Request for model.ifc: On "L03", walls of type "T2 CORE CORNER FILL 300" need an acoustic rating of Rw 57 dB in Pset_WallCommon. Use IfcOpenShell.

First a look at what the model holds.

```python
import ifcopenshell
import ifcopenshell.util.element

model = ifcopenshell.open("model.ifc")
print(model.schema)
storey = next(s for s in model.by_type("IfcBuildingStorey") if s.Name == "L03")
walls = [e for e in ifcopenshell.util.element.get_decomposition(storey) if e.is_a("IfcWall")]
seen = {}
for e in walls:
    element_type = ifcopenshell.util.element.get_type(e)
    key = (element_type.Name if element_type != e and element_type else None, ifcopenshell.util.element.get_pset(e, "Pset_WallCommon", "AcousticRating"))
    seen[key] = seen.get(key, 0) + 1
for (name, value), count in sorted(seen.items(), key=str):
    print(count, "x", name, "|", value)
```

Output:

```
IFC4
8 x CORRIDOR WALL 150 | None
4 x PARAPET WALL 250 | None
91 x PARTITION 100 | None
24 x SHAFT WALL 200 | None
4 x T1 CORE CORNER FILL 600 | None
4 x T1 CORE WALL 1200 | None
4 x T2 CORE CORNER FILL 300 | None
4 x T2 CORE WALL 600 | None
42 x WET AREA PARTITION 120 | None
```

```python
import ifcopenshell
import ifcopenshell.api.pset
import ifcopenshell.util.element

model = ifcopenshell.open("model.ifc")

storey = next(s for s in model.by_type("IfcBuildingStorey") if s.Name == "L03")
walls = [e for e in ifcopenshell.util.element.get_decomposition(storey) if e.is_a("IfcWall")]

count = 0
for e in walls:
    element_type = ifcopenshell.util.element.get_type(e)
    if element_type in (None, e) or element_type.Name != "T2 CORE CORNER FILL 300":
        continue
    found = ifcopenshell.util.element.get_pset(e, "Pset_WallCommon", should_inherit=False)
    if found:
        pset = model.by_id(found["id"])
        if len(ifcopenshell.util.element.get_elements_by_pset(pset)) > 1:
            pset = ifcopenshell.api.pset.unshare_pset(model, products=[e], pset=pset)[0]
    else:
        pset = ifcopenshell.api.pset.add_pset(model, product=e, name="Pset_WallCommon")
    ifcopenshell.api.pset.edit_pset(model, pset=pset, properties={"AcousticRating": "Rw 57 dB"})
    count += 1

print(count, "walls updated")

model.write("model_rev.ifc")
```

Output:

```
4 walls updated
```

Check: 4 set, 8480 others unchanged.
